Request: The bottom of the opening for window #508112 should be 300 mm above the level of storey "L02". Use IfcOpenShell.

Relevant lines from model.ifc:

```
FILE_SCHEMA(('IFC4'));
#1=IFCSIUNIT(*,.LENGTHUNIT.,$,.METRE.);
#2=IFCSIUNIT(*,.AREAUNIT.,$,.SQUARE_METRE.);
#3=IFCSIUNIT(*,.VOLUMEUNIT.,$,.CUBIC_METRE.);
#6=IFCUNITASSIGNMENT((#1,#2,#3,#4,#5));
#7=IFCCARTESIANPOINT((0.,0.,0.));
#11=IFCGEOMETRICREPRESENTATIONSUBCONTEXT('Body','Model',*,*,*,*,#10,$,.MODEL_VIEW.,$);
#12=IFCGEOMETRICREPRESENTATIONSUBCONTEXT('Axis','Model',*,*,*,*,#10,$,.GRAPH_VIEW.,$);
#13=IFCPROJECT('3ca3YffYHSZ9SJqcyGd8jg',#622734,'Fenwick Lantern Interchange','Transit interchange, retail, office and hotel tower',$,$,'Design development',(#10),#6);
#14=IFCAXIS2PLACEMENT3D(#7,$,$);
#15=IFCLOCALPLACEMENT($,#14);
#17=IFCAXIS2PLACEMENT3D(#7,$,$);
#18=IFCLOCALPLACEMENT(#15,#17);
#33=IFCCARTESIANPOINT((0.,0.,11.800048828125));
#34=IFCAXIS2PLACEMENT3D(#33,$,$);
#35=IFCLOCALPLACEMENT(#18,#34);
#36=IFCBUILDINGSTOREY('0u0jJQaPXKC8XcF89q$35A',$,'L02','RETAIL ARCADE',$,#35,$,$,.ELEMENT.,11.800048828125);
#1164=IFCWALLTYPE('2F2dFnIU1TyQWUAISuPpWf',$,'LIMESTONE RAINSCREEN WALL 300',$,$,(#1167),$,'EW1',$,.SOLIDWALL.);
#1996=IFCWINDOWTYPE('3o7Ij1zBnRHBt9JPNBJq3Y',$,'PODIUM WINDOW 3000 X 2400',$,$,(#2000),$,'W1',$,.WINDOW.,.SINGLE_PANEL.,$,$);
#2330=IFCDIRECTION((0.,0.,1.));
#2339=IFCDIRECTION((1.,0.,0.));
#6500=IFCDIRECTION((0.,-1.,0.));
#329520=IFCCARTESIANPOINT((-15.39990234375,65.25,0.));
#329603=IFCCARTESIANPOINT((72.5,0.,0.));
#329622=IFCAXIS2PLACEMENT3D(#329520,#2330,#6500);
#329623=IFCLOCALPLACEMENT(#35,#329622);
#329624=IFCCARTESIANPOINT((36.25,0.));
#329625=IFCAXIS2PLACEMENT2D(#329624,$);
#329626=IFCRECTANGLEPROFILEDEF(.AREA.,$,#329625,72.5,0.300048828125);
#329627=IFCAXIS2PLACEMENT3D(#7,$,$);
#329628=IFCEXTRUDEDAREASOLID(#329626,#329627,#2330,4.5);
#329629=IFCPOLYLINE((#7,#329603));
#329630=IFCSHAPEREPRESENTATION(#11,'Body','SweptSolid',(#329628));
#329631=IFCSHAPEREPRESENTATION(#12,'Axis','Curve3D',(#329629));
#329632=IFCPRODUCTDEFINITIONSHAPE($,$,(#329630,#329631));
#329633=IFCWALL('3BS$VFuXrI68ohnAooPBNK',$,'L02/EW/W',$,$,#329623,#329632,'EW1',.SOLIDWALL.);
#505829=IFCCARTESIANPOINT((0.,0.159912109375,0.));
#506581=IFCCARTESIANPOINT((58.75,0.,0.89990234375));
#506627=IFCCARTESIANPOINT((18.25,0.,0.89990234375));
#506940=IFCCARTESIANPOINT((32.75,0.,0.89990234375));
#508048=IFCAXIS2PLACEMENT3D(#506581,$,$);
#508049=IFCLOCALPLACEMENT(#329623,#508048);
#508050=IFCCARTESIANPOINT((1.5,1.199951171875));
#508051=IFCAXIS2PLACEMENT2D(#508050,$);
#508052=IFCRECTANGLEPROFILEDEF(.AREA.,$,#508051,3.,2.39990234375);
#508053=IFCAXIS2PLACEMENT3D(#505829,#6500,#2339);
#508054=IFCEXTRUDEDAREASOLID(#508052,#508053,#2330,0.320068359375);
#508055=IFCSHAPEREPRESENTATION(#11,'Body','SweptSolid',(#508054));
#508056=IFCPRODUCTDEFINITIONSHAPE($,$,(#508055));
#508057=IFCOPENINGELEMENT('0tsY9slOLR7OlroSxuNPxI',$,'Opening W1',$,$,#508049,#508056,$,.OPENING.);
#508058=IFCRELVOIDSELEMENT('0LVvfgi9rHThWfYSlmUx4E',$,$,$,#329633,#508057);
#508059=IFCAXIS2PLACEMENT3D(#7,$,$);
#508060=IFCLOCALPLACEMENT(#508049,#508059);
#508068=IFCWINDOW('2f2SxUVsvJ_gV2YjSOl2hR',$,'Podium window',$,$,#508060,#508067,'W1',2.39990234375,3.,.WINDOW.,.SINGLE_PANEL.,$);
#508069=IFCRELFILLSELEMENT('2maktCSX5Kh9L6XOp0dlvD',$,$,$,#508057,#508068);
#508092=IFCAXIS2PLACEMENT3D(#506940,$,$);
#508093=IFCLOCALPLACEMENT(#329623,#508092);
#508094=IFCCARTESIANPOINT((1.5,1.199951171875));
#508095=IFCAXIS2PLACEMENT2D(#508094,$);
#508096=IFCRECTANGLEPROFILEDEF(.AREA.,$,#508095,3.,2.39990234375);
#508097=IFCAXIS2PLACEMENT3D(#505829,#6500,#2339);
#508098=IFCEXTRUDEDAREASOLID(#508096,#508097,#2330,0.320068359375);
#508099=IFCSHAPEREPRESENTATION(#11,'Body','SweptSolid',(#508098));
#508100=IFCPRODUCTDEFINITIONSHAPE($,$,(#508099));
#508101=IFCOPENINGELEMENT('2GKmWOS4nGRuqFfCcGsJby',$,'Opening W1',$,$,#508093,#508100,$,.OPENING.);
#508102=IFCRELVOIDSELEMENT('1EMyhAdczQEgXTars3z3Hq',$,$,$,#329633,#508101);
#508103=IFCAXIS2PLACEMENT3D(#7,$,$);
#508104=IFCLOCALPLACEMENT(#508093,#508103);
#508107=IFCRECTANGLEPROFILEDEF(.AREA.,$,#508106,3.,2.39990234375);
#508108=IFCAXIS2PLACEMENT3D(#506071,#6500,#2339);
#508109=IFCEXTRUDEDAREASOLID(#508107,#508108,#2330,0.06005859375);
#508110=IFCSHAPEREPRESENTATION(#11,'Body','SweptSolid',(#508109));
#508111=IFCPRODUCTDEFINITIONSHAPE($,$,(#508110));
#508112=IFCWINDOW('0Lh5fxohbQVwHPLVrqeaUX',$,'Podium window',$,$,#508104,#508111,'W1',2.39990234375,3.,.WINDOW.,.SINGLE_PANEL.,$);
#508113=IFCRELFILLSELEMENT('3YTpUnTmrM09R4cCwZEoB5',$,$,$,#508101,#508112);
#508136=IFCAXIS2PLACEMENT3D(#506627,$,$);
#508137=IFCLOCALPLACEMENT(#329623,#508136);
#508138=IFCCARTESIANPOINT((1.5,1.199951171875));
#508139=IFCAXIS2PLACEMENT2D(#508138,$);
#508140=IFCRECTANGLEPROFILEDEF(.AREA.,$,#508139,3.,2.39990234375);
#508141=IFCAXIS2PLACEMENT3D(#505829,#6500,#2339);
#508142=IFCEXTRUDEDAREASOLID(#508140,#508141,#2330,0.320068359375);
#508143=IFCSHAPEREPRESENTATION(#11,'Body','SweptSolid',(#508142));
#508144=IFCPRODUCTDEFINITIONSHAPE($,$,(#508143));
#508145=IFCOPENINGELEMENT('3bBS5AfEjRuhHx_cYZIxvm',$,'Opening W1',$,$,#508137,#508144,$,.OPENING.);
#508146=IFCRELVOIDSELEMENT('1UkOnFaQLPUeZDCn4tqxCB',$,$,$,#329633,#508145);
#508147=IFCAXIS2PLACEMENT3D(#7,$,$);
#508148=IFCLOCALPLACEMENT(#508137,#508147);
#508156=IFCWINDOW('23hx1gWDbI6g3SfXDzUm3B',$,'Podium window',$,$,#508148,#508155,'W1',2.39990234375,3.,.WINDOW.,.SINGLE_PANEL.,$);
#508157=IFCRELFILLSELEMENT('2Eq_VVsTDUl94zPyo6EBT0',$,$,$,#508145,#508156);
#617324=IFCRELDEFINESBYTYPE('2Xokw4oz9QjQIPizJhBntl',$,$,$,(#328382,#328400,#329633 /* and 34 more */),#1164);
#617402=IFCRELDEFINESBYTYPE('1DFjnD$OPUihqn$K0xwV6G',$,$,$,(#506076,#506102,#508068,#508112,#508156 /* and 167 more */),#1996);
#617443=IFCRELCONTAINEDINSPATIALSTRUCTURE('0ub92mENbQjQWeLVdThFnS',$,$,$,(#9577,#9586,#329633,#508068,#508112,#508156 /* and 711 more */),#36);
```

```python
import numpy as np
import ifcopenshell
import ifcopenshell.api.geometry
import ifcopenshell.geom
import ifcopenshell.util.element
import ifcopenshell.util.placement
import ifcopenshell.util.shape
import ifcopenshell.util.unit

model = ifcopenshell.open("model.ifc")
unit_scale = ifcopenshell.util.unit.calculate_unit_scale(model)

window = model.by_guid("0Lh5fxohbQVwHPLVrqeaUX")
opening = window.FillsVoids[0].RelatingOpeningElement
storey = ifcopenshell.util.element.get_container(window, ifc_class="IfcBuildingStorey")
level = ifcopenshell.util.placement.get_local_placement(storey.ObjectPlacement)[2, 3]

# The opening's origin need not be at the sill, so measure its lowest point.
shape = ifcopenshell.geom.create_shape(ifcopenshell.geom.settings(), opening)
bottom = ifcopenshell.util.shape.get_shape_bottom_elevation(shape, shape.geometry) / unit_scale
dz = level + 0.3 / unit_scale - bottom

shift = np.array([0.0, 0.0, dz])
# The window is placed relative to its opening, so it follows when the opening moves.
matrix = ifcopenshell.util.placement.get_local_placement(opening.ObjectPlacement)
matrix[:3, 3] += shift
ifcopenshell.api.geometry.edit_object_placement(
    model, product=opening, matrix=matrix, is_si=False, should_transform_children=True
)

print(f"moved by {dz * unit_scale:+.3f} m")

model.write("model-out.ifc")
```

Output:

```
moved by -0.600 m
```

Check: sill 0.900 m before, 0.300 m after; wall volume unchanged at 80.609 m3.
